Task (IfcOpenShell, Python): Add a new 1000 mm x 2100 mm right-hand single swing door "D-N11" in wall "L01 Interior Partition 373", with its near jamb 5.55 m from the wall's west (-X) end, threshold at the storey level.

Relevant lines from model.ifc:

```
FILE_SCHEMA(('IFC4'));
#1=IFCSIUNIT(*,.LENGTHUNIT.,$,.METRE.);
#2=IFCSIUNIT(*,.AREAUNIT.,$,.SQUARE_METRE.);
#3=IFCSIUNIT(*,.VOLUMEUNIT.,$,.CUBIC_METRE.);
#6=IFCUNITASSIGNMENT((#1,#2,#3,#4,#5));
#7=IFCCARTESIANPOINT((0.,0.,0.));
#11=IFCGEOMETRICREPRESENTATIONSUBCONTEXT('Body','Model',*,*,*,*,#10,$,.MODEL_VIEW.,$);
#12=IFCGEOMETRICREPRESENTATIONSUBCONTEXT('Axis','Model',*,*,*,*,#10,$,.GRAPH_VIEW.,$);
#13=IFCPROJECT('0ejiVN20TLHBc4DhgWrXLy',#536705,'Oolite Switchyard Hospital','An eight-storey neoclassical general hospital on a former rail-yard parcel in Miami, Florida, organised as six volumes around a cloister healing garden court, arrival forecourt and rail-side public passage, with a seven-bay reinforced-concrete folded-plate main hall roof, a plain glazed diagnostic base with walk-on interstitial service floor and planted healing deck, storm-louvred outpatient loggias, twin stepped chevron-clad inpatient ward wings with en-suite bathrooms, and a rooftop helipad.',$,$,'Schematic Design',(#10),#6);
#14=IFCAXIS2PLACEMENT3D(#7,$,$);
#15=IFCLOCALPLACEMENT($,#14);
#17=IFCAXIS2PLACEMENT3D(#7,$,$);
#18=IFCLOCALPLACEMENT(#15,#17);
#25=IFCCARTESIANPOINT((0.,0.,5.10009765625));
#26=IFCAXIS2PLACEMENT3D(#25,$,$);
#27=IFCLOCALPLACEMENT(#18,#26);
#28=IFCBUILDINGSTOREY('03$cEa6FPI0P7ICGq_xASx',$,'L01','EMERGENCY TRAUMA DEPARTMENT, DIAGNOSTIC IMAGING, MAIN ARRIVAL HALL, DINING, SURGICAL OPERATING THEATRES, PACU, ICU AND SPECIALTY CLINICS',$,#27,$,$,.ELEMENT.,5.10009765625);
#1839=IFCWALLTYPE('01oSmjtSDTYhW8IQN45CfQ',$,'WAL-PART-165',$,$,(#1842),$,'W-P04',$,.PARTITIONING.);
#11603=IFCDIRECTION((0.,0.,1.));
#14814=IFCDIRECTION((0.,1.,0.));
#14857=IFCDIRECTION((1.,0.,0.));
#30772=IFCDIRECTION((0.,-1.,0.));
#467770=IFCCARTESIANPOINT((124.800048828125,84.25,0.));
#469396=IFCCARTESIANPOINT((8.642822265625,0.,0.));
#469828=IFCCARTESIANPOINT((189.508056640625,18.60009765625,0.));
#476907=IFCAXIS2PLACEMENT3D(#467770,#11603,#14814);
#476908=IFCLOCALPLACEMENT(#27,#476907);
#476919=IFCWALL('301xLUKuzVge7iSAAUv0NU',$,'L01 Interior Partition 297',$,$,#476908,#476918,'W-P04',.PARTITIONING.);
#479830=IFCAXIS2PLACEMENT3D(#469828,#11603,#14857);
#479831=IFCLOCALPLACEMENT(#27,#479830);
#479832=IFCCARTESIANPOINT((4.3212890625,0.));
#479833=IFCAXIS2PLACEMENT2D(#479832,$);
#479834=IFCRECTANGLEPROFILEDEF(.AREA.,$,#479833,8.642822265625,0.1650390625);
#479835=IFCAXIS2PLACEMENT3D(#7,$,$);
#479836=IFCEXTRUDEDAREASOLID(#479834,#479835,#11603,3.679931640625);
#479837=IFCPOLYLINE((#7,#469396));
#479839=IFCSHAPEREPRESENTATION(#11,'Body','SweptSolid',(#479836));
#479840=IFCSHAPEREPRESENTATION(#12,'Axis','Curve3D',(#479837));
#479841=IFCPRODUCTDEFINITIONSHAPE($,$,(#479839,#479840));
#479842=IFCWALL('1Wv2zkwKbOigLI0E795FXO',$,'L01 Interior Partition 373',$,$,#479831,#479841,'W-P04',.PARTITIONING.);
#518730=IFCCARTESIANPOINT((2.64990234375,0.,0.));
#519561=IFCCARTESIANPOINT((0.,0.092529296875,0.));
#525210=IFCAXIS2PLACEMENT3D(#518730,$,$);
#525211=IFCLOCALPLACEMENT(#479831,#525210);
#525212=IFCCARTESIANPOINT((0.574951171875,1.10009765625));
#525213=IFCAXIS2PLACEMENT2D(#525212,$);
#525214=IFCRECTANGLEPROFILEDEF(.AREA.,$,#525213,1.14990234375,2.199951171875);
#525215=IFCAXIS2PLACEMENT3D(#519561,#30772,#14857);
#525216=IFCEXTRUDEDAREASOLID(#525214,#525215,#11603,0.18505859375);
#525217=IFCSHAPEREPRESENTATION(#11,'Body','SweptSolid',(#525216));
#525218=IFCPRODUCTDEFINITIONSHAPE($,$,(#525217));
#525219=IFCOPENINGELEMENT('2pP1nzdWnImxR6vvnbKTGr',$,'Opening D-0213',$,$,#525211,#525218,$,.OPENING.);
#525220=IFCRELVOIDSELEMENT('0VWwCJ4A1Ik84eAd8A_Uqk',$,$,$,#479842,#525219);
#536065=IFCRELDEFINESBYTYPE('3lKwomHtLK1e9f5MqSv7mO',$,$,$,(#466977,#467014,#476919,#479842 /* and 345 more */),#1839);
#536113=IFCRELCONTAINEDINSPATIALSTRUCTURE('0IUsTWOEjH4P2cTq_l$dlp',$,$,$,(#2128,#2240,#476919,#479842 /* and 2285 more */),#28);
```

```python
import numpy as np
import ifcopenshell
import ifcopenshell.api.feature
import ifcopenshell.api.geometry
import ifcopenshell.api.root
import ifcopenshell.api.spatial
import ifcopenshell.geom
import ifcopenshell.util.element
import ifcopenshell.util.placement
import ifcopenshell.util.representation
import ifcopenshell.util.shape
import ifcopenshell.util.unit

model = ifcopenshell.open("model.ifc")
unit_scale = ifcopenshell.util.unit.calculate_unit_scale(model)
settings = ifcopenshell.geom.settings()


def volume(element):
    """Net volume in cubic metres, openings subtracted."""
    shape = ifcopenshell.geom.create_shape(settings, element)
    return ifcopenshell.util.shape.get_volume(shape.geometry)


wall = model.by_guid("1Wv2zkwKbOigLI0E795FXO")
storey = ifcopenshell.util.element.get_container(wall, ifc_class="IfcBuildingStorey")
context = ifcopenshell.util.representation.get_context(model, "Model", "Body", "MODEL_VIEW")
before = volume(wall)

width, height, from_end, sill = 1, 2.1, 5.55, 0.0  # metres

# The wall runs along its own X axis, and the end named is its -X end.
wall_shape = ifcopenshell.geom.create_shape(settings, wall)
x, y, z = ifcopenshell.util.shape.get_vertices(wall_shape.geometry).T
start = x.min() + from_end
face, thickness = float(y.min()), float(y.max() - y.min())
wall_matrix = ifcopenshell.util.placement.get_local_placement(wall.ObjectPlacement)
level = ifcopenshell.util.placement.get_local_placement(storey.ObjectPlacement)[2, 3]


def in_wall(x, y):
    """Placement at x, y metres in the wall's axes, at sill height."""
    matrix = wall_matrix.copy()
    matrix[:, 3] = wall_matrix @ np.array([x / unit_scale, y / unit_scale, 0.0, 1.0])
    matrix[2, 3] = level + sill / unit_scale
    return matrix


# Opening: a box that overshoots both wall faces by 50 mm.
opening = ifcopenshell.api.root.create_entity(model, ifc_class="IfcOpeningElement", predefined_type="OPENING")
box = ifcopenshell.api.geometry.add_wall_representation(
    model, context=context, length=width, height=height, thickness=thickness + 0.1
)
ifcopenshell.api.geometry.assign_representation(model, product=opening, representation=box)
ifcopenshell.api.geometry.edit_object_placement(model, product=opening, matrix=in_wall(start, face - 0.05), is_si=False)
ifcopenshell.api.feature.add_feature(model, feature=opening, element=wall)

door = ifcopenshell.api.root.create_entity(model, ifc_class="IfcDoor", name="D-N11", predefined_type="DOOR")
door.OverallWidth, door.OverallHeight = width / unit_scale, height / unit_scale
door.OperationType = "SINGLE_SWING_RIGHT"
body = ifcopenshell.api.geometry.add_door_representation(
    model,
    context=context,
    overall_width=door.OverallWidth,
    overall_height=door.OverallHeight,
    operation_type="SINGLE_SWING_RIGHT",
    lining_properties={"LiningDepth": thickness / unit_scale, "ThresholdDepth": thickness / unit_scale},
)
ifcopenshell.api.geometry.assign_representation(model, product=door, representation=body)
ifcopenshell.api.spatial.assign_container(model, products=[door], relating_structure=storey)
ifcopenshell.api.feature.add_filling(model, opening=opening, element=door)

# The lining spans the wall, so the door starts at the wall face.
ifcopenshell.api.geometry.edit_object_placement(model, product=door, matrix=in_wall(start, face), is_si=False)

after = volume(wall)

print(f"wall volume {before:.3f} -> {after:.3f} m3")

model.write("model_updated.ifc")
```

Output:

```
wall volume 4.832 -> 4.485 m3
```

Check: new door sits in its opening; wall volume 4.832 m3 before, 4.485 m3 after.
